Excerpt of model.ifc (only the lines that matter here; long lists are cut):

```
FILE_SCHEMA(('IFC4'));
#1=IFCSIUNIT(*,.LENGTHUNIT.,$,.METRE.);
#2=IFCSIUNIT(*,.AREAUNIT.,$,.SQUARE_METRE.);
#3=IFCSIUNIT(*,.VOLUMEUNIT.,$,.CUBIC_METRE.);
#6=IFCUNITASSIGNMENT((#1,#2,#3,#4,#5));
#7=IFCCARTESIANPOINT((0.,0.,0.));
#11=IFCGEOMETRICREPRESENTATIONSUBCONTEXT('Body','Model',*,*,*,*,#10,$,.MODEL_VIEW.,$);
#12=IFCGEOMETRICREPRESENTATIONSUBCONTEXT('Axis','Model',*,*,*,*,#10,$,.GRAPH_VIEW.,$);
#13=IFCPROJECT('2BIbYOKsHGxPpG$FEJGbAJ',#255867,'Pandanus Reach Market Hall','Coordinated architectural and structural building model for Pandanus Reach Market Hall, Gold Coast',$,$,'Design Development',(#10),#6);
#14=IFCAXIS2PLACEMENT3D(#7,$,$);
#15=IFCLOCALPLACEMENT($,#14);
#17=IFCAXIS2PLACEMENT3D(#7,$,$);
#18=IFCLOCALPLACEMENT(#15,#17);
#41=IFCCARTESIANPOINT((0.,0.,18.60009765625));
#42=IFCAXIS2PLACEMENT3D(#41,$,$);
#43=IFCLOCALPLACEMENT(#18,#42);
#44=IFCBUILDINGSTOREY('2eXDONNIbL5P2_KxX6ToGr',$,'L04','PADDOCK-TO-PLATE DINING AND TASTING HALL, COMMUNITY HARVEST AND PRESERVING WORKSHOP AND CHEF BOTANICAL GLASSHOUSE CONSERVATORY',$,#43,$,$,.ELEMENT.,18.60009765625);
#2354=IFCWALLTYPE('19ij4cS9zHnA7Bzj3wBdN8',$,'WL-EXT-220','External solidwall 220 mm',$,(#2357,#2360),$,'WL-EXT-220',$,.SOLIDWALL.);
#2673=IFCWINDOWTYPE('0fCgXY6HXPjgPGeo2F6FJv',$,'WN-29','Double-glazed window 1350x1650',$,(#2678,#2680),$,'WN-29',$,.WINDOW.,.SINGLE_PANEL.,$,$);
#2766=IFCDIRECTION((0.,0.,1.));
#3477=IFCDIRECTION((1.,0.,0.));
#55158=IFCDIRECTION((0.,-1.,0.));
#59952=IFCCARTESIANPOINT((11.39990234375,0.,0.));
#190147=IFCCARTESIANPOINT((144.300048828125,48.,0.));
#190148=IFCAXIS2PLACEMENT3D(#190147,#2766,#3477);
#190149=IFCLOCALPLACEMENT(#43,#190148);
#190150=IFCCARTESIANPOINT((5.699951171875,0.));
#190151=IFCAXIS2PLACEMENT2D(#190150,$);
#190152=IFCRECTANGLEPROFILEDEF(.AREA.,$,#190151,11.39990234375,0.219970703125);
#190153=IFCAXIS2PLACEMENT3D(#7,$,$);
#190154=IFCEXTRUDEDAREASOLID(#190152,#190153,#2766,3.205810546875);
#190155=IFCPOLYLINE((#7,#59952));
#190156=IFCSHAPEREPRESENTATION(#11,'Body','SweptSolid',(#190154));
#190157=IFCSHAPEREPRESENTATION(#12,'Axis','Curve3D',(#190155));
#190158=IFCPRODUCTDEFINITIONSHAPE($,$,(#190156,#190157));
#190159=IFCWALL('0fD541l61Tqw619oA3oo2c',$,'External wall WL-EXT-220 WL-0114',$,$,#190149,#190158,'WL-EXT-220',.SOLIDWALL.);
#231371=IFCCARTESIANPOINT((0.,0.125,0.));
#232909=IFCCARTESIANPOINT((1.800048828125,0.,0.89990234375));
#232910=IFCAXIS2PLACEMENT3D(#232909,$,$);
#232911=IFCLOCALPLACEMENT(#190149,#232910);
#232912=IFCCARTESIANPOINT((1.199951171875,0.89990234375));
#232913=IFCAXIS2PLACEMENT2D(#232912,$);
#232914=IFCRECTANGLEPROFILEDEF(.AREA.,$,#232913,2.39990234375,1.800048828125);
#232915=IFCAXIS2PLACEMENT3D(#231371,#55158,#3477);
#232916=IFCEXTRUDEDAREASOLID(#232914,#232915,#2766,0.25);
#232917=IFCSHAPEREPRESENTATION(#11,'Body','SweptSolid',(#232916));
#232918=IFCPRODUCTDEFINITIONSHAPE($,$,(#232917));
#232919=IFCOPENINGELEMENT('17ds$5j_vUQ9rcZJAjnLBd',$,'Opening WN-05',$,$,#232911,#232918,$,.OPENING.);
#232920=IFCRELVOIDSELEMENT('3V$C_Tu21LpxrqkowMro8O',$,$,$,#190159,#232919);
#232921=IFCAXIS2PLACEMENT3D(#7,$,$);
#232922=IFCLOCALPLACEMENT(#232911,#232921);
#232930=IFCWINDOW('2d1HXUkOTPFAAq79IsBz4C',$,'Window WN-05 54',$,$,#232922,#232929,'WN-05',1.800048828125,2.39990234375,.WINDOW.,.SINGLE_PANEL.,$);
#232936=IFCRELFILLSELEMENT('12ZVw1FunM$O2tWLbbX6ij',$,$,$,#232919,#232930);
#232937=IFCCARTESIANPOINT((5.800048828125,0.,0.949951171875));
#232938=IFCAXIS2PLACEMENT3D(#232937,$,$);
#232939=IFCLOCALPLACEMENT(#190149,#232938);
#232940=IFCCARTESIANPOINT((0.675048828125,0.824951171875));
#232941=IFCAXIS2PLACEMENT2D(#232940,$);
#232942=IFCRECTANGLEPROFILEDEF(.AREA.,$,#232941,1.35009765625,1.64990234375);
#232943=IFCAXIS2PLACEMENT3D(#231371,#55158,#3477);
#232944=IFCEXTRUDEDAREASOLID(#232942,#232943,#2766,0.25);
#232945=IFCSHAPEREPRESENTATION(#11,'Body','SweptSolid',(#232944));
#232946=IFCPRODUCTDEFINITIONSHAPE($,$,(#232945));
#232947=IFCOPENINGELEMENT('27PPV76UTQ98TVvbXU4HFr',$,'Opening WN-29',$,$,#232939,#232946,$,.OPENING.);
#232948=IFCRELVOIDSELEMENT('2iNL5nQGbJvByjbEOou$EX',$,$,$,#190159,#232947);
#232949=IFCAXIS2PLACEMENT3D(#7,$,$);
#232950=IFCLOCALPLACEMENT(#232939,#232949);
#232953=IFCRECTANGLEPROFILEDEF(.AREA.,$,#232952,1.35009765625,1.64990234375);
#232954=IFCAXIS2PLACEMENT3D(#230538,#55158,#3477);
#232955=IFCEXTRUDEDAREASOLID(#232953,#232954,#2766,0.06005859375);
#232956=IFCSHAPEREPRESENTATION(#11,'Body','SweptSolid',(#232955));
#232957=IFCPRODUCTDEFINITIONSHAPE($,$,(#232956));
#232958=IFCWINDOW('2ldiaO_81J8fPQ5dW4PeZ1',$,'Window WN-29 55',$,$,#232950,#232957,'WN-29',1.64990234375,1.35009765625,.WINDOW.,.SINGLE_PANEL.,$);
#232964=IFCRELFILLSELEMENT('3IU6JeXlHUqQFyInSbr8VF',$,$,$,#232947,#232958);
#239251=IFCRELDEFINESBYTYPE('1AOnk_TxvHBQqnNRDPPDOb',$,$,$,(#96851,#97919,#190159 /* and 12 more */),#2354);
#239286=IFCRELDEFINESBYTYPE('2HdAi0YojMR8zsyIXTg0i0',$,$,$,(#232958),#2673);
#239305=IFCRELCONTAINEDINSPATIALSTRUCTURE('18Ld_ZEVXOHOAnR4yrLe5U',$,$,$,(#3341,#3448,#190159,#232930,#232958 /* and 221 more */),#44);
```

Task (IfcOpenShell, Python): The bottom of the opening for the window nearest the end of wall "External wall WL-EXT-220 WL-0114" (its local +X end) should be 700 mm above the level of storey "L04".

```python
import numpy as np
import ifcopenshell
import ifcopenshell.api.geometry
import ifcopenshell.geom
import ifcopenshell.util.element
import ifcopenshell.util.placement
import ifcopenshell.util.shape
import ifcopenshell.util.unit

model = ifcopenshell.open("model.ifc")
unit_scale = ifcopenshell.util.unit.calculate_unit_scale(model)

window = model.by_guid("2ldiaO_81J8fPQ5dW4PeZ1")
opening = window.FillsVoids[0].RelatingOpeningElement
storey = ifcopenshell.util.element.get_container(window, ifc_class="IfcBuildingStorey")
level = ifcopenshell.util.placement.get_local_placement(storey.ObjectPlacement)[2, 3]

# The opening's origin need not be at the sill, so measure its lowest point.
shape = ifcopenshell.geom.create_shape(ifcopenshell.geom.settings(), opening)
bottom = ifcopenshell.util.shape.get_shape_bottom_elevation(shape, shape.geometry) / unit_scale
dz = level + 0.7 / unit_scale - bottom

shift = np.array([0.0, 0.0, dz])
# The window is placed relative to its opening, so it follows when the opening moves.
matrix = ifcopenshell.util.placement.get_local_placement(opening.ObjectPlacement)
matrix[:3, 3] += shift
ifcopenshell.api.geometry.edit_object_placement(
    model, product=opening, matrix=matrix, is_si=False, should_transform_children=True
)

print(f"moved by {dz * unit_scale:+.3f} m")

model.write("model-out.ifc")
```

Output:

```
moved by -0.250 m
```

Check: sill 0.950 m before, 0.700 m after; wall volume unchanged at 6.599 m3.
